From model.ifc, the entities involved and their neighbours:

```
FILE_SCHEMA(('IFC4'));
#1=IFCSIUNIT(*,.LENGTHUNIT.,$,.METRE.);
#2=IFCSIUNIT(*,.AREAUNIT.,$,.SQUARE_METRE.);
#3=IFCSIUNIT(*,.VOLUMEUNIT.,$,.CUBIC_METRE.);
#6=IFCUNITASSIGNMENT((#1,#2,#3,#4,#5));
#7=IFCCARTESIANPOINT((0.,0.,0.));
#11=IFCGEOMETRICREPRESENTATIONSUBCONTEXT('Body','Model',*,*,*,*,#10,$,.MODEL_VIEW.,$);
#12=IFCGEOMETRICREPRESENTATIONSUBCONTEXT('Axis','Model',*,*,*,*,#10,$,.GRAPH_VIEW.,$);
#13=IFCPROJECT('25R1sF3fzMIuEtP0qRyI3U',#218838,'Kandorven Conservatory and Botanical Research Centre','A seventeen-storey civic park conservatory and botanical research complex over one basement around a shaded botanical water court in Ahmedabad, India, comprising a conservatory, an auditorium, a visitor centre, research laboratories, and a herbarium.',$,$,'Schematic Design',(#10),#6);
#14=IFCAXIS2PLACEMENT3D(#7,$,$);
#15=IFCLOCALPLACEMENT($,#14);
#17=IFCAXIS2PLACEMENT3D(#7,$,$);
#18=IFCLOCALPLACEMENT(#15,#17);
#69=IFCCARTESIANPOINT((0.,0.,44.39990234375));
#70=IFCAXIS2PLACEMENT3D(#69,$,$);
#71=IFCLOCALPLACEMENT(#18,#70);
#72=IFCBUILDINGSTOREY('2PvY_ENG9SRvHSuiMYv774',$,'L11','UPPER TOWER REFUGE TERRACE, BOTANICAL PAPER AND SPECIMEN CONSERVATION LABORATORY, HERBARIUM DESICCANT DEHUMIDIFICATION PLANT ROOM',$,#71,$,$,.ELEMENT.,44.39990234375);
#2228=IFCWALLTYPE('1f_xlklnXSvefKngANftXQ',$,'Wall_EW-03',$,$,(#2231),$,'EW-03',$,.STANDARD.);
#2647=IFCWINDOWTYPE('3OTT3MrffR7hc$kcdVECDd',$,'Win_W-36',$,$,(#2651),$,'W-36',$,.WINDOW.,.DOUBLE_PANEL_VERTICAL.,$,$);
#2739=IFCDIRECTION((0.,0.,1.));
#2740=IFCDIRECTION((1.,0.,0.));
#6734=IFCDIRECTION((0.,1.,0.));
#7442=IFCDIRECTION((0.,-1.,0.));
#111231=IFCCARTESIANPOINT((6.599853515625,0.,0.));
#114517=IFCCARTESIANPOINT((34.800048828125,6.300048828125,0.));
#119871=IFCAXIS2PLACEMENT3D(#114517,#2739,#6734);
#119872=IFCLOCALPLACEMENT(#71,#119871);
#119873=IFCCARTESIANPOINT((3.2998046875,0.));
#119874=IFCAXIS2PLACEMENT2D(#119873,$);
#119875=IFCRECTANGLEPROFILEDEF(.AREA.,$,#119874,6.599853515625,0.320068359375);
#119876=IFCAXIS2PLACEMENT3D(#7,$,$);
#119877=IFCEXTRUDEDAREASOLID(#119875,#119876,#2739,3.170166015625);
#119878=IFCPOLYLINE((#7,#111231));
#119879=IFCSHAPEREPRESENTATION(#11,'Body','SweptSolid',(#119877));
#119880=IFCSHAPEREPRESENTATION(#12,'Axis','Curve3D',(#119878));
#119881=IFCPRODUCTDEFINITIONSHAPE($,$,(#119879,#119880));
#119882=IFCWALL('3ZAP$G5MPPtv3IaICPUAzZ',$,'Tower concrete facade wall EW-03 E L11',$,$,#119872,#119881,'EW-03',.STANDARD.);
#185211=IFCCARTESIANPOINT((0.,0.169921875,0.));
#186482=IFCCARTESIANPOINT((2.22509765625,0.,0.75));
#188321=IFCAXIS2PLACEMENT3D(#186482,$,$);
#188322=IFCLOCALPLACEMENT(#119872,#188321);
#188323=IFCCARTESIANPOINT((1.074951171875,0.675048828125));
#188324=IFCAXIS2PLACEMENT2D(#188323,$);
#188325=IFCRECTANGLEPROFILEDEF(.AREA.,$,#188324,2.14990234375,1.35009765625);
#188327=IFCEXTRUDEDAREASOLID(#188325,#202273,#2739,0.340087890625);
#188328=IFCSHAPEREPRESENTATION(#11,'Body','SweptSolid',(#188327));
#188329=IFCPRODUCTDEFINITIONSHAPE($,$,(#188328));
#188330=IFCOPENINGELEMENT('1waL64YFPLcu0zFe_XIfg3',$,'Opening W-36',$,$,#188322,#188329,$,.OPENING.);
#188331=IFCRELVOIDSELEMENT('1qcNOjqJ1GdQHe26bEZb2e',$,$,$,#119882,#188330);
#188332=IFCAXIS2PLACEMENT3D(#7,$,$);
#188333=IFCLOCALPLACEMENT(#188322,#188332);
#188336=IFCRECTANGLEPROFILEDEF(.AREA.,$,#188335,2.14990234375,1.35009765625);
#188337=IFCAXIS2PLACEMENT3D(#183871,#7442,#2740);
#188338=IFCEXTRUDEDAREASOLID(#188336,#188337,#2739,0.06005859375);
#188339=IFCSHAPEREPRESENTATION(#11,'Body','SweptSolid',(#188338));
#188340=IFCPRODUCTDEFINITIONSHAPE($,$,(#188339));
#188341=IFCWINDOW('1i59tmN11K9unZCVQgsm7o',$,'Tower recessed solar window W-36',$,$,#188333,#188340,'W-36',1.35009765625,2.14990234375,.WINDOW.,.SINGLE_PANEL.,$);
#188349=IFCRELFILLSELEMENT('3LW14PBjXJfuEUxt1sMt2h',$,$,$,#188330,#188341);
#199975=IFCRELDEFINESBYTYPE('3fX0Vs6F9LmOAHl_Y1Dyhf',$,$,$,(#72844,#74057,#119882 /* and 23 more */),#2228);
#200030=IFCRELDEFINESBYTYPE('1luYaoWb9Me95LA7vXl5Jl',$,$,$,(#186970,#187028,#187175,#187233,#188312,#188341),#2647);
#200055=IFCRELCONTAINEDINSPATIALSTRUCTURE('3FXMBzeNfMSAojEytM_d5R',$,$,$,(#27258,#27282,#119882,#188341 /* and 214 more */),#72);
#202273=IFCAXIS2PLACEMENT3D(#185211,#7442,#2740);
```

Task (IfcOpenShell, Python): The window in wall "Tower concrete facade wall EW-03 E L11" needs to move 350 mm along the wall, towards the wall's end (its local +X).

```python
import ifcopenshell
import ifcopenshell.api.geometry
import ifcopenshell.util.placement
import ifcopenshell.util.unit

model = ifcopenshell.open("model.ifc")
unit_scale = ifcopenshell.util.unit.calculate_unit_scale(model)

window = model.by_id(188341)
opening = window.FillsVoids[0].RelatingOpeningElement
wall = opening.VoidsElements[0].RelatingBuildingElement

wall_matrix = ifcopenshell.util.placement.get_local_placement(wall.ObjectPlacement)
shift = wall_matrix[:3, 0] * 0.35 / unit_scale
before = ifcopenshell.util.placement.get_local_placement(window.ObjectPlacement)[:3, 3].copy()

# The window is placed relative to its opening, so it follows when the opening moves.
matrix = ifcopenshell.util.placement.get_local_placement(opening.ObjectPlacement)
matrix[:3, 3] += shift
ifcopenshell.api.geometry.edit_object_placement(
    model, product=opening, matrix=matrix, is_si=False, should_transform_children=True
)

after = ifcopenshell.util.placement.get_local_placement(window.ObjectPlacement)[:3, 3]
print("window moved by", (after - before).round(3) + 0.0)

model.write("model_updated.ifc")
```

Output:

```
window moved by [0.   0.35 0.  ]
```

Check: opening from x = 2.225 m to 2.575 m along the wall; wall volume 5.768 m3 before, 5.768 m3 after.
